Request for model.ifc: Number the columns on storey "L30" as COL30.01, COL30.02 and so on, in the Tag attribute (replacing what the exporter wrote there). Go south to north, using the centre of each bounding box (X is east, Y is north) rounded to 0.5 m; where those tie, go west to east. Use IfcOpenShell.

First a look at what the model holds.

```python
import ifcopenshell
import ifcopenshell.util.element
import ifcopenshell.util.placement

model = ifcopenshell.open("model.ifc")
print(model.schema)
storey = next(s for s in model.by_type("IfcBuildingStorey") if s.Name == "L30")
columns = [e for e in ifcopenshell.util.element.get_decomposition(storey) if e.is_a("IfcColumn")]
for e in sorted(columns, key=lambda e: e.id()):
    origin = ifcopenshell.util.placement.get_local_placement(e.ObjectPlacement)[:3, 3]
    print(e.id(), e.Tag, e.Name, origin.round(2) + 0.0, sep=" | ")
```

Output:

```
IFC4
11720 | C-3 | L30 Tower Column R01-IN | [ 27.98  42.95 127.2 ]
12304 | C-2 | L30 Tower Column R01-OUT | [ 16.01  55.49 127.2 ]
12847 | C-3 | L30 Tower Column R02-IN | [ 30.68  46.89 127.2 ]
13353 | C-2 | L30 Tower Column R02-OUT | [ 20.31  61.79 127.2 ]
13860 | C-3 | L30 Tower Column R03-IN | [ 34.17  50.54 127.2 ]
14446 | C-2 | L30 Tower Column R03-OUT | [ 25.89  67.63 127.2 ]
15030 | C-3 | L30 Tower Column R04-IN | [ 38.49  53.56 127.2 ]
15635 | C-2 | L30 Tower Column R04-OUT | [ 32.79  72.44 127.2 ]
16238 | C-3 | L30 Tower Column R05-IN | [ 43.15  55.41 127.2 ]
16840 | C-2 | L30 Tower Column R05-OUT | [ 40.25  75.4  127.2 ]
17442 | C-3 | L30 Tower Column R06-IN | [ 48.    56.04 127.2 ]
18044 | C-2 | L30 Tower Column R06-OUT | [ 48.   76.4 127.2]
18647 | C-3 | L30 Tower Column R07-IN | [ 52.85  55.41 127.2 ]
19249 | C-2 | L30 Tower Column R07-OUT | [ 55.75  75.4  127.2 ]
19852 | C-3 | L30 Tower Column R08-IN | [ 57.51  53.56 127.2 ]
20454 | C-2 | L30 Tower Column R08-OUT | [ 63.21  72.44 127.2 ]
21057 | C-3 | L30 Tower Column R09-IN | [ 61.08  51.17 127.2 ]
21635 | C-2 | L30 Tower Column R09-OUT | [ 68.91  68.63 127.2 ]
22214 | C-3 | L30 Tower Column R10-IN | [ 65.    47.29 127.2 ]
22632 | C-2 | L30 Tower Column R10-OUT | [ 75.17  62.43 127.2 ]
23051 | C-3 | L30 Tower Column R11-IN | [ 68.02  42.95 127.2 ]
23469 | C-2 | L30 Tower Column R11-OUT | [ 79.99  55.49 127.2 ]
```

```python
import ifcopenshell
import ifcopenshell.geom
import ifcopenshell.util.element
import ifcopenshell.util.shape

model = ifcopenshell.open("model.ifc")
settings = ifcopenshell.geom.settings()
settings.set("use-world-coords", True)


def centre(element):
    shape = ifcopenshell.geom.create_shape(settings, element)
    return ifcopenshell.util.shape.get_bbox_centroid(shape.geometry)


storey = next(s for s in model.by_type("IfcBuildingStorey") if s.Name == "L30")
columns = [e for e in ifcopenshell.util.element.get_decomposition(storey) if e.is_a("IfcColumn")]

# Insertion points can sit at a corner or the storey origin, so sort by the geometry (in metres).
centres = {e: centre(e) for e in columns}
columns.sort(key=lambda e: (round(centres[e][1] / 0.5), centres[e][0]))

for i, e in enumerate(columns, start=1):
    number = f"COL30.{i:02d}"
    e.Tag = number
    print(e.id(), number)

model.write("model_v2.ifc")
```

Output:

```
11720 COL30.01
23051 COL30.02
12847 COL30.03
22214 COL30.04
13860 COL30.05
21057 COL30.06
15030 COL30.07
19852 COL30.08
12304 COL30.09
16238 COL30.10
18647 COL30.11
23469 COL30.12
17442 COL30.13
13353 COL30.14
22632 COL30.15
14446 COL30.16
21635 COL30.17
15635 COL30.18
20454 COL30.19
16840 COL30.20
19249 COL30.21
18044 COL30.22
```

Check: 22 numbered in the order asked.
